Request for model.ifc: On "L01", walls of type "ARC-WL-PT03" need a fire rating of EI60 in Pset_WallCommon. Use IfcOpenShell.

First a look at what the model holds.

```python
import ifcopenshell
import ifcopenshell.util.element

model = ifcopenshell.open("model.ifc")
print(model.schema)
storey = next(s for s in model.by_type("IfcBuildingStorey") if s.Name == "L01")
walls = [e for e in ifcopenshell.util.element.get_decomposition(storey) if e.is_a("IfcWall")]
seen = {}
for e in walls:
    element_type = ifcopenshell.util.element.get_type(e)
    key = (element_type.Name if element_type != e and element_type else None, ifcopenshell.util.element.get_pset(e, "Pset_WallCommon", "FireRating"))
    seen[key] = seen.get(key, 0) + 1
for (name, value), count in sorted(seen.items(), key=str):
    print(count, "x", name, "|", value)
```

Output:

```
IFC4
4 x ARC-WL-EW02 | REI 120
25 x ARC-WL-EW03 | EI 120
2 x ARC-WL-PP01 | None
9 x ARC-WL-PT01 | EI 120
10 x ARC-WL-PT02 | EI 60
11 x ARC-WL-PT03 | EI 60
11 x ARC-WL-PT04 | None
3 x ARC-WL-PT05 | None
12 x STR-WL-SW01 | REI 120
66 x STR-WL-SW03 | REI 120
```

```python
import ifcopenshell
import ifcopenshell.api.pset
import ifcopenshell.util.element

model = ifcopenshell.open("model.ifc")

storey = next(s for s in model.by_type("IfcBuildingStorey") if s.Name == "L01")
walls = [e for e in ifcopenshell.util.element.get_decomposition(storey) if e.is_a("IfcWall")]

count = 0
for e in walls:
    element_type = ifcopenshell.util.element.get_type(e)
    if element_type in (None, e) or element_type.Name != "ARC-WL-PT03":
        continue
    # add_pset returns the element's existing set when there is one.
    pset = ifcopenshell.api.pset.add_pset(model, product=e, name="Pset_WallCommon")
    ifcopenshell.api.pset.edit_pset(model, pset=pset, properties={"FireRating": "EI60"})
    count += 1

print(count, "walls updated")

model.write("model_edited.ifc")
```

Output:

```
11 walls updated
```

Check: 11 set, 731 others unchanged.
